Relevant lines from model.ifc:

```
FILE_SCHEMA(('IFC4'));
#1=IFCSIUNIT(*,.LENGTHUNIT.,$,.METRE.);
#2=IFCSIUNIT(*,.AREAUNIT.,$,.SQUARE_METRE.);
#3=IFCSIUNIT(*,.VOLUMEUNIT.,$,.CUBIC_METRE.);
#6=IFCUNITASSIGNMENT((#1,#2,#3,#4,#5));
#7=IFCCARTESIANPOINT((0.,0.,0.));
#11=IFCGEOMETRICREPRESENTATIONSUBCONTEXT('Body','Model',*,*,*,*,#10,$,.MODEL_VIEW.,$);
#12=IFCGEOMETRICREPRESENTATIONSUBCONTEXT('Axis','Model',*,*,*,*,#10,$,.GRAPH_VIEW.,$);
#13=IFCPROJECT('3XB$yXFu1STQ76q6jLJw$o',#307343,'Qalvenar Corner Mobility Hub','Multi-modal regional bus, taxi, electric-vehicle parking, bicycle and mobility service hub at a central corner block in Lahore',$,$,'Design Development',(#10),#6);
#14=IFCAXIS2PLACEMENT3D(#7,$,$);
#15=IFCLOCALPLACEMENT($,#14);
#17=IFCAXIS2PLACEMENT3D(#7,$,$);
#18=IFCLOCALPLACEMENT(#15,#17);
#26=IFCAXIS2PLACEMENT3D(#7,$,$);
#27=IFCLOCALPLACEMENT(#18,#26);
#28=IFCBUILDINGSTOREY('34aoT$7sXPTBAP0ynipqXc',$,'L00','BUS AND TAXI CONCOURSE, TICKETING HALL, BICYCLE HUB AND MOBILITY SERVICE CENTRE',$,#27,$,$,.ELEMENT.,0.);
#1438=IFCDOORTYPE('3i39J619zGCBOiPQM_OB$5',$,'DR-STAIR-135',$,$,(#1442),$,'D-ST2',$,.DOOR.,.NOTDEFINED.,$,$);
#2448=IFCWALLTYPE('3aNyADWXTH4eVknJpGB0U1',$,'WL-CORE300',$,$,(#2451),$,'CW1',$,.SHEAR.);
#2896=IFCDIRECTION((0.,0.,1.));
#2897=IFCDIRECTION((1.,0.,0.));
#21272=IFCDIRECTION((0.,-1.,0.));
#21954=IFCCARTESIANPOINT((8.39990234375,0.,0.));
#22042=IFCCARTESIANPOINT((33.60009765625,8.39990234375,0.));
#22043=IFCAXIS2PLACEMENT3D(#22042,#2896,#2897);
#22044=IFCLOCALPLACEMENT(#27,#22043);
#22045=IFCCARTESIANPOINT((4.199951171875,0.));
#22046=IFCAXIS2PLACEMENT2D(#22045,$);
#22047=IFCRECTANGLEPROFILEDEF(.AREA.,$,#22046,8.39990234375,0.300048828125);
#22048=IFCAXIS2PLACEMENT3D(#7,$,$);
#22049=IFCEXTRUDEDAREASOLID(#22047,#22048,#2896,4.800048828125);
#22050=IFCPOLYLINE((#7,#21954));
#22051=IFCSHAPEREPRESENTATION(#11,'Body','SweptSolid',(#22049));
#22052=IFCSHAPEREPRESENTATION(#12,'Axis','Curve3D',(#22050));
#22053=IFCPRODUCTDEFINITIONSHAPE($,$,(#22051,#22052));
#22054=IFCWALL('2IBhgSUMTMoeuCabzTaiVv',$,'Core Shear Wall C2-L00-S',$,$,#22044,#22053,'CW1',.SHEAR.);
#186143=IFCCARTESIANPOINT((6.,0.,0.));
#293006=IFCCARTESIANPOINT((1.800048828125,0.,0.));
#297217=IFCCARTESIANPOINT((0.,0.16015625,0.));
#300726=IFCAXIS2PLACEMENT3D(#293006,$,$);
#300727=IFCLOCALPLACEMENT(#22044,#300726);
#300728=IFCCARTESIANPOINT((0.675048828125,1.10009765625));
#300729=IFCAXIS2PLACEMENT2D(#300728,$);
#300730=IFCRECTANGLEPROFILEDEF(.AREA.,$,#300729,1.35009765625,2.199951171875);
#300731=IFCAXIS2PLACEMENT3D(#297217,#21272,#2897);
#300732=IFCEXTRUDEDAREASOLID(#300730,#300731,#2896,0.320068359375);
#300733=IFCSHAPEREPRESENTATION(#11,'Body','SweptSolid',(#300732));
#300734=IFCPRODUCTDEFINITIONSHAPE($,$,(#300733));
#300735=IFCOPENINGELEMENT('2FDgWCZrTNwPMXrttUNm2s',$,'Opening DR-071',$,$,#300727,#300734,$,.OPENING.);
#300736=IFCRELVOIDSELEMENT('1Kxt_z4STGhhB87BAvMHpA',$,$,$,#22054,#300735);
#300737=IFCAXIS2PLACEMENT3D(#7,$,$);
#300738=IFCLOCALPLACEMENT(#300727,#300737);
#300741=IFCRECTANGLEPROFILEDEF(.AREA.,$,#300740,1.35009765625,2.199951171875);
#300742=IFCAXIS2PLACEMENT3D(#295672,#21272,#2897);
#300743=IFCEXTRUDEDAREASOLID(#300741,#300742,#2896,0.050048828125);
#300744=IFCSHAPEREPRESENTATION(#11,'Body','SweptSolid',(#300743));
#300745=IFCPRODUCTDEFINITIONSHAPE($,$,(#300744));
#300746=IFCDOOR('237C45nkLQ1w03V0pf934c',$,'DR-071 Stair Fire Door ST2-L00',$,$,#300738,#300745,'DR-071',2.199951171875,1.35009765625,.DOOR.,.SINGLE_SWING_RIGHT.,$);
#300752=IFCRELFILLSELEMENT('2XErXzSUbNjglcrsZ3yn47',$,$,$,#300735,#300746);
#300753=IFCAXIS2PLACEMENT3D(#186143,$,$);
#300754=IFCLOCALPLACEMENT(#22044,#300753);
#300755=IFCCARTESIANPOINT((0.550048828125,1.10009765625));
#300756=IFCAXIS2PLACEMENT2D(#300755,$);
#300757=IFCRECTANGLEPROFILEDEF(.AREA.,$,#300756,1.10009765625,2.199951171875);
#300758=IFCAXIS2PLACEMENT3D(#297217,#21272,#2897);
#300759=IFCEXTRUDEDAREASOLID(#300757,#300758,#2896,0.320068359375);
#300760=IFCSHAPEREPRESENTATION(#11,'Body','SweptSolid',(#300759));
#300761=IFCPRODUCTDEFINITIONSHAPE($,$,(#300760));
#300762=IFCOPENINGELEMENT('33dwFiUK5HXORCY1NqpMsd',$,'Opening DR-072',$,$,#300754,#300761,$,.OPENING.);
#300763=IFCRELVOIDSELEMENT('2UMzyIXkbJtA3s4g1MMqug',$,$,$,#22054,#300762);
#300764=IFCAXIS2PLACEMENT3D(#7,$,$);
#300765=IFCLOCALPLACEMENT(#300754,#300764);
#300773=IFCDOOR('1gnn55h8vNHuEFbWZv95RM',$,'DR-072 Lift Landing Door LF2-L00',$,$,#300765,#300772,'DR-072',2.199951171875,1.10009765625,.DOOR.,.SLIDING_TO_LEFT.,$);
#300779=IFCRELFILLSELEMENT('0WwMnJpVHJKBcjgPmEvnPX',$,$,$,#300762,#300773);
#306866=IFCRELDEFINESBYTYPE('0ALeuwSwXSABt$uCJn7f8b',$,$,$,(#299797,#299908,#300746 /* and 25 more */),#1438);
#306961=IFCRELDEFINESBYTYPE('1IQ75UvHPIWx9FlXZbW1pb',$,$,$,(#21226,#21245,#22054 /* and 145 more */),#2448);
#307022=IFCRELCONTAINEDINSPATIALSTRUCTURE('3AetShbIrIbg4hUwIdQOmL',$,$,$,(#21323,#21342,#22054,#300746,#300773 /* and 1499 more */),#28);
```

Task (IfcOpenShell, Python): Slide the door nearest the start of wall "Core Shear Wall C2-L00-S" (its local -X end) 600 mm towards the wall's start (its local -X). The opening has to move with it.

```python
import ifcopenshell
import ifcopenshell.api.geometry
import ifcopenshell.util.placement
import ifcopenshell.util.unit

model = ifcopenshell.open("model.ifc")
unit_scale = ifcopenshell.util.unit.calculate_unit_scale(model)

door = model.by_id(300746)
opening = door.FillsVoids[0].RelatingOpeningElement
wall = opening.VoidsElements[0].RelatingBuildingElement

wall_matrix = ifcopenshell.util.placement.get_local_placement(wall.ObjectPlacement)
shift = wall_matrix[:3, 0] * -0.6 / unit_scale
before = ifcopenshell.util.placement.get_local_placement(door.ObjectPlacement)[:3, 3].copy()

# The door is placed relative to its opening, so it follows when the opening moves.
matrix = ifcopenshell.util.placement.get_local_placement(opening.ObjectPlacement)
matrix[:3, 3] += shift
ifcopenshell.api.geometry.edit_object_placement(
    model, product=opening, matrix=matrix, is_si=False, should_transform_children=True
)

after = ifcopenshell.util.placement.get_local_placement(door.ObjectPlacement)[:3, 3]
print("door moved by", (after - before).round(3) + 0.0)

model.write("model-out.ifc")
```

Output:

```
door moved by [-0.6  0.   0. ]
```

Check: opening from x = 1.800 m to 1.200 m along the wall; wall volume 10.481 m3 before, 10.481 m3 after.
